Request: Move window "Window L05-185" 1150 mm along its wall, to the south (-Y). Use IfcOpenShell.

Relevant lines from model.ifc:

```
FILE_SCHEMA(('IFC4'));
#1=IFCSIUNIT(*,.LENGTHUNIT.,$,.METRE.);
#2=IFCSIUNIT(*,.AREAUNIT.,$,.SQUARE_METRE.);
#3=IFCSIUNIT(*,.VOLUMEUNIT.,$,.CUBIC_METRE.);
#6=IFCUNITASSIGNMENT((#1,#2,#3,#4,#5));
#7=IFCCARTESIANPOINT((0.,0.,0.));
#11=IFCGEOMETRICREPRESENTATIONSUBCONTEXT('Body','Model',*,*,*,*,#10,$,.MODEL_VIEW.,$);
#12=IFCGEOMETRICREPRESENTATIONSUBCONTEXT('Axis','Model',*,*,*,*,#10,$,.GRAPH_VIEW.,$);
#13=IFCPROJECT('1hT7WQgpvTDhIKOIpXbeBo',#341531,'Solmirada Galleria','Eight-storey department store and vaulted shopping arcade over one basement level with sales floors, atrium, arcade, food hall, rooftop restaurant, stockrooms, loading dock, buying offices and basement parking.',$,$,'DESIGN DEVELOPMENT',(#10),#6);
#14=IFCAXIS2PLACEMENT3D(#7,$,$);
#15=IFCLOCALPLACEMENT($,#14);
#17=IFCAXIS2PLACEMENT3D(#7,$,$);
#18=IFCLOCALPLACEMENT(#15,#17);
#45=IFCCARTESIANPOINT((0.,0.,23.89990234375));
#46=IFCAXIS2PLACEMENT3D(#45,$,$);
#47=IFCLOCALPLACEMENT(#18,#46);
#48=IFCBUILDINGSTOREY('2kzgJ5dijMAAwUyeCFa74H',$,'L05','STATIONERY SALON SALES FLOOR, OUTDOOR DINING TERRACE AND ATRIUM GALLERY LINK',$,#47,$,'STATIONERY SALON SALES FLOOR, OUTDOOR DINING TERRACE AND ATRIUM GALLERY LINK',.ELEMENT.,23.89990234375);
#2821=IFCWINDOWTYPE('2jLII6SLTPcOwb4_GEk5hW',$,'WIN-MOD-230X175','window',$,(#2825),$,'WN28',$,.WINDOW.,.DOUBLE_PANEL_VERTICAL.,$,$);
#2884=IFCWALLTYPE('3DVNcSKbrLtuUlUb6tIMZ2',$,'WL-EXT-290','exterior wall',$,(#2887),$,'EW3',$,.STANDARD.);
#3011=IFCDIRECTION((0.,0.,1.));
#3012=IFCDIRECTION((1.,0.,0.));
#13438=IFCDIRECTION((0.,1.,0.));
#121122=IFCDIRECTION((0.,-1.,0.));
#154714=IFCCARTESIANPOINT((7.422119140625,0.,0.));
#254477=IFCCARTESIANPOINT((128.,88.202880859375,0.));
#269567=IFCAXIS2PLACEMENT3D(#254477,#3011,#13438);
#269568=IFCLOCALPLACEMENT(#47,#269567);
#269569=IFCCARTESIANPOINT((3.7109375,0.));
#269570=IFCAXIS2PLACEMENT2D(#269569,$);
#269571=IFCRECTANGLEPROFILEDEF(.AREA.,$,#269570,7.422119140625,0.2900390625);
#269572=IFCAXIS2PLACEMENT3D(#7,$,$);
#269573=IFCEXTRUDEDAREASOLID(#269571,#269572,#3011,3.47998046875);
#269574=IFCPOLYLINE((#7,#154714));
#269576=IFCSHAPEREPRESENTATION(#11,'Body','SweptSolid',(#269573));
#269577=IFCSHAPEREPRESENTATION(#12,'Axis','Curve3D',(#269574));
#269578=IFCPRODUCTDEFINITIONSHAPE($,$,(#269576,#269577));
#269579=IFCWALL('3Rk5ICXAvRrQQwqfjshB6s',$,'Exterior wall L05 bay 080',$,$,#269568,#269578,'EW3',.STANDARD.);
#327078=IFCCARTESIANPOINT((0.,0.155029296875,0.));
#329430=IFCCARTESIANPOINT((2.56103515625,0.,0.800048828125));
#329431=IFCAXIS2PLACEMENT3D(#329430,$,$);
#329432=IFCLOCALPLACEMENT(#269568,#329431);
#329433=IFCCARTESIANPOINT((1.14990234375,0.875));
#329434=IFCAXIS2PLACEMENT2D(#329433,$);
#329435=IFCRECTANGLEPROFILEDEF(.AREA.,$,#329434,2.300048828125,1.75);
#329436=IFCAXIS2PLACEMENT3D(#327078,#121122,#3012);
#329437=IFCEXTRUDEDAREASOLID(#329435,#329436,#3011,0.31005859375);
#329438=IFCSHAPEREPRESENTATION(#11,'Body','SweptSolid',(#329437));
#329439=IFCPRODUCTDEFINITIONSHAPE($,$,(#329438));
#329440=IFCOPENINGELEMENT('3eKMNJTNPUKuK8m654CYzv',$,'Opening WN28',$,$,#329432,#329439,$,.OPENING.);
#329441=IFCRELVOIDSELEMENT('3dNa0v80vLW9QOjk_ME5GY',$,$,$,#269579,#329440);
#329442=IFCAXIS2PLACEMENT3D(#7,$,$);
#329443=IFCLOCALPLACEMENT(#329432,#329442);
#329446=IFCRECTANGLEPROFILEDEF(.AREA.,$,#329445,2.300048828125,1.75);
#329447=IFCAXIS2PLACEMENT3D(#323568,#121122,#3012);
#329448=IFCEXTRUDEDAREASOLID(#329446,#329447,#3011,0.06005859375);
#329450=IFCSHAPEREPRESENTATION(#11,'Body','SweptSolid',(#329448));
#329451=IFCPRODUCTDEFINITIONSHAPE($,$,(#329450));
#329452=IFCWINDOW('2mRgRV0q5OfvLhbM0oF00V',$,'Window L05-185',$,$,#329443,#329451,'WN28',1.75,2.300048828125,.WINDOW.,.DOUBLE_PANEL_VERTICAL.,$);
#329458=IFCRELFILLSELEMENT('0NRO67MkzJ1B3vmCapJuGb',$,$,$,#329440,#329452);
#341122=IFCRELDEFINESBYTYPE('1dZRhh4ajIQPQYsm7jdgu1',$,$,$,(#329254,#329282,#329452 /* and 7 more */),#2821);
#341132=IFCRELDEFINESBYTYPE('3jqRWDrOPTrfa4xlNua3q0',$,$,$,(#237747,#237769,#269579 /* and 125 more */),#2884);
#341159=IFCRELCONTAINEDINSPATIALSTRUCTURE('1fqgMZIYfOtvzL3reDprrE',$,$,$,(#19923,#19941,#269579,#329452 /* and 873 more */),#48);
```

```python
import ifcopenshell
import ifcopenshell.api.geometry
import ifcopenshell.util.placement
import ifcopenshell.util.unit

model = ifcopenshell.open("model.ifc")
unit_scale = ifcopenshell.util.unit.calculate_unit_scale(model)

window = model.by_guid("2mRgRV0q5OfvLhbM0oF00V")
opening = window.FillsVoids[0].RelatingOpeningElement
wall = opening.VoidsElements[0].RelatingBuildingElement

wall_matrix = ifcopenshell.util.placement.get_local_placement(wall.ObjectPlacement)
shift = wall_matrix[:3, 0] * -1.15 / unit_scale
before = ifcopenshell.util.placement.get_local_placement(window.ObjectPlacement)[:3, 3].copy()

# The window is placed relative to its opening, so it follows when the opening moves.
matrix = ifcopenshell.util.placement.get_local_placement(opening.ObjectPlacement)
matrix[:3, 3] += shift
ifcopenshell.api.geometry.edit_object_placement(
    model, product=opening, matrix=matrix, is_si=False, should_transform_children=True
)

after = ifcopenshell.util.placement.get_local_placement(window.ObjectPlacement)[:3, 3]
print("window moved by", (after - before).round(3) + 0.0)

model.write("model_edited.ifc")
```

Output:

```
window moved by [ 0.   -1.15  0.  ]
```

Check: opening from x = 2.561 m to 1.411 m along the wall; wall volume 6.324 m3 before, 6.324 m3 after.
